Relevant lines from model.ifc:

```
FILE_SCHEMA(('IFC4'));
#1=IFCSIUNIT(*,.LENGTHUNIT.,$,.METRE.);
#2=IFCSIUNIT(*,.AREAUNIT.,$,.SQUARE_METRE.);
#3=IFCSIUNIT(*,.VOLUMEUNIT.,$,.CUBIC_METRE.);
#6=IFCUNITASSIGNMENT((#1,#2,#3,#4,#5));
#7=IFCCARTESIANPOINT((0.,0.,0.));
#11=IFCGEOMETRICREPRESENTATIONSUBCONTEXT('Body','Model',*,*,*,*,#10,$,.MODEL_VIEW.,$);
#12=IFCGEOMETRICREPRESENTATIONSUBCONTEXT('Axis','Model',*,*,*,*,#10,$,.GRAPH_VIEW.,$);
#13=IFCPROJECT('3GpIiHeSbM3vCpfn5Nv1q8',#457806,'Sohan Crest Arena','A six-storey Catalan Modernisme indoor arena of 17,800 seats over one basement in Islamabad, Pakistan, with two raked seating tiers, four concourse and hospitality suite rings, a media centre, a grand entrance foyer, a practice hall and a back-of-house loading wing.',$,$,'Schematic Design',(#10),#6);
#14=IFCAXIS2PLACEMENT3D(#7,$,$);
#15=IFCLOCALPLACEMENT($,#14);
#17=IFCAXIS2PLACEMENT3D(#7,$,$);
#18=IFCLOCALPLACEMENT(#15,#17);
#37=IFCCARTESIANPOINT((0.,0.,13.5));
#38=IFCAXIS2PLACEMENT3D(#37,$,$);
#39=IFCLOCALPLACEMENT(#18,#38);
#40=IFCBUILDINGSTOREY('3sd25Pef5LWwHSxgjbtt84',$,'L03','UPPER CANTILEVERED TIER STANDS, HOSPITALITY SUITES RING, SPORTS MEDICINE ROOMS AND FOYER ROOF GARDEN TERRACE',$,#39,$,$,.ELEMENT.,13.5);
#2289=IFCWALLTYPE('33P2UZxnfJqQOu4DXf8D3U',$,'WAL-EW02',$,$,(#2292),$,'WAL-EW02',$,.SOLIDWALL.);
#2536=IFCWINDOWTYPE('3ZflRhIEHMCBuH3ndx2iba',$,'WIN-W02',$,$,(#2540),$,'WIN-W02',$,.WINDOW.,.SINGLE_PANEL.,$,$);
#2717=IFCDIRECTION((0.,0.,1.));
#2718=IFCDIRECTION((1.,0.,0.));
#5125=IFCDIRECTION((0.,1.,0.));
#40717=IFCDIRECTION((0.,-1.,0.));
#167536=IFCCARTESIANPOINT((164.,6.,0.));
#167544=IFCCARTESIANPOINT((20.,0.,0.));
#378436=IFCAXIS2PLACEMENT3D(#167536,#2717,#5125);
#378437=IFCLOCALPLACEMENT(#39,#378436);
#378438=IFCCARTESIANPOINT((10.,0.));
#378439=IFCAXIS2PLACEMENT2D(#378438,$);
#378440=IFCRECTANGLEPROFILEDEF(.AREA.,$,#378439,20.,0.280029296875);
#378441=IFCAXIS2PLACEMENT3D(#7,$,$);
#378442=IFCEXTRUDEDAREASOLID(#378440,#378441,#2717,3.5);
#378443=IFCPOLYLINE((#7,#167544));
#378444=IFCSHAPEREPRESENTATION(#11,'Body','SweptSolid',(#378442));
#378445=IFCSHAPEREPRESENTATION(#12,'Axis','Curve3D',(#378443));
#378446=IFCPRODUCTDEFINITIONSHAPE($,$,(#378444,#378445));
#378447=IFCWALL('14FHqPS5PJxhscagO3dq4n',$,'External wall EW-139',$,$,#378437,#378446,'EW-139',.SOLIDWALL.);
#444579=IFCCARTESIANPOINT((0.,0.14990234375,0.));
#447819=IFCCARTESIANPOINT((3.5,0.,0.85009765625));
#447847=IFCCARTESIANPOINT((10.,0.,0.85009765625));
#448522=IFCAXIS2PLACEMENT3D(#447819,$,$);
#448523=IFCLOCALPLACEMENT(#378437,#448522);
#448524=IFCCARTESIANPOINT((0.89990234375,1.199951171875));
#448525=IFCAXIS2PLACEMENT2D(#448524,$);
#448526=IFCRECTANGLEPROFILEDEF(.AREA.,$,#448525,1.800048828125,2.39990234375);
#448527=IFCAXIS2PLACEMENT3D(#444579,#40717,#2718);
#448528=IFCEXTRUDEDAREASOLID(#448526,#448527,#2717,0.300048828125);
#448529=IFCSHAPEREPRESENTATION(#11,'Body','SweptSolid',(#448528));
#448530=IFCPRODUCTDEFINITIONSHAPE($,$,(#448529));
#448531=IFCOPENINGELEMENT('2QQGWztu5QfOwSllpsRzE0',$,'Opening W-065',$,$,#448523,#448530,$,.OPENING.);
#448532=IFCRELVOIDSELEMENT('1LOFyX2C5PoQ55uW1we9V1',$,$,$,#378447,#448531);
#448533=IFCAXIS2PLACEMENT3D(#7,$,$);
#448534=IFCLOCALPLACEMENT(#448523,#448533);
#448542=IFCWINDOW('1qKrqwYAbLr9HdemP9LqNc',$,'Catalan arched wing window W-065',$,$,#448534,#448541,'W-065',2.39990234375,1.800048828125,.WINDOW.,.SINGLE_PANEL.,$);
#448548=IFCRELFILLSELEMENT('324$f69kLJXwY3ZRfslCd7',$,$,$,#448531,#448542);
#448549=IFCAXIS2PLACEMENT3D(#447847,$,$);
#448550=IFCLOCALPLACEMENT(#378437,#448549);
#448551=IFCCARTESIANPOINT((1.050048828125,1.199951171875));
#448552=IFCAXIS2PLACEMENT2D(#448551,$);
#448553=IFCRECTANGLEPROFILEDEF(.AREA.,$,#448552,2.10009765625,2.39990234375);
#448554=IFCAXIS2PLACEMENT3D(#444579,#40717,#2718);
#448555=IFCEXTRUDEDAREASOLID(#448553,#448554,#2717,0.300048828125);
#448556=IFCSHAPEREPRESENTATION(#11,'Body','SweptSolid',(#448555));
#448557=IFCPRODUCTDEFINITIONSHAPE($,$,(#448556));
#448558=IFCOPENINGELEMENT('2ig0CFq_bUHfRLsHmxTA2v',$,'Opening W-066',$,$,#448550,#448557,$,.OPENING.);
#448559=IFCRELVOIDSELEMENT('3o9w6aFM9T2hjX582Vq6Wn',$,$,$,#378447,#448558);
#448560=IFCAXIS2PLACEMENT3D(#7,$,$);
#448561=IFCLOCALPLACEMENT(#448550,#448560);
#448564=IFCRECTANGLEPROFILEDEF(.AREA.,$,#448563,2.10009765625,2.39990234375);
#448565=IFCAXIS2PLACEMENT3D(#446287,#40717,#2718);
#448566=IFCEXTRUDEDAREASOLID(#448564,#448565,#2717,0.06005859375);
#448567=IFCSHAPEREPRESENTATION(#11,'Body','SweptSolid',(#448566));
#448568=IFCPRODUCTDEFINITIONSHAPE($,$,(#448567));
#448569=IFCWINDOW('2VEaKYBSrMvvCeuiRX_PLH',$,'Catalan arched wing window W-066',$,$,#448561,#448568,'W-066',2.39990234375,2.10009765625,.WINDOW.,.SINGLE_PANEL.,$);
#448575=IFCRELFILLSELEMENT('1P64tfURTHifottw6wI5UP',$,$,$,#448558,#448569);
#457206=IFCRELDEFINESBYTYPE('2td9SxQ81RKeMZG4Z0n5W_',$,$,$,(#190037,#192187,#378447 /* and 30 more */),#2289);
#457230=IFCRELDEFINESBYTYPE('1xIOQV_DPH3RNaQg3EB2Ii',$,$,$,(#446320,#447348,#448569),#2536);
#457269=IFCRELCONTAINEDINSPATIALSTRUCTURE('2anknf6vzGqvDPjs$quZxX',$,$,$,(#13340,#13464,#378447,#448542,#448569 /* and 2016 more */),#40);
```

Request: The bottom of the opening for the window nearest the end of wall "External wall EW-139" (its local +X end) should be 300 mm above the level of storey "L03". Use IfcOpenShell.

```python
import numpy as np
import ifcopenshell
import ifcopenshell.api.geometry
import ifcopenshell.geom
import ifcopenshell.util.element
import ifcopenshell.util.placement
import ifcopenshell.util.shape
import ifcopenshell.util.unit

model = ifcopenshell.open("model.ifc")
unit_scale = ifcopenshell.util.unit.calculate_unit_scale(model)

window = model.by_guid("2VEaKYBSrMvvCeuiRX_PLH")
opening = window.FillsVoids[0].RelatingOpeningElement
storey = ifcopenshell.util.element.get_container(window, ifc_class="IfcBuildingStorey")
level = ifcopenshell.util.placement.get_local_placement(storey.ObjectPlacement)[2, 3]

# The opening's origin need not be at the sill, so measure its lowest point.
shape = ifcopenshell.geom.create_shape(ifcopenshell.geom.settings(), opening)
bottom = ifcopenshell.util.shape.get_shape_bottom_elevation(shape, shape.geometry) / unit_scale
dz = level + 0.3 / unit_scale - bottom

shift = np.array([0.0, 0.0, dz])
# The window is placed relative to its opening, so it follows when the opening moves.
matrix = ifcopenshell.util.placement.get_local_placement(opening.ObjectPlacement)
matrix[:3, 3] += shift
ifcopenshell.api.geometry.edit_object_placement(
    model, product=opening, matrix=matrix, is_si=False, should_transform_children=True
)

print(f"moved by {dz * unit_scale:+.3f} m")

model.write("model_v2.ifc")
```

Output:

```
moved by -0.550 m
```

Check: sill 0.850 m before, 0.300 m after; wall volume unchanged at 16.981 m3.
